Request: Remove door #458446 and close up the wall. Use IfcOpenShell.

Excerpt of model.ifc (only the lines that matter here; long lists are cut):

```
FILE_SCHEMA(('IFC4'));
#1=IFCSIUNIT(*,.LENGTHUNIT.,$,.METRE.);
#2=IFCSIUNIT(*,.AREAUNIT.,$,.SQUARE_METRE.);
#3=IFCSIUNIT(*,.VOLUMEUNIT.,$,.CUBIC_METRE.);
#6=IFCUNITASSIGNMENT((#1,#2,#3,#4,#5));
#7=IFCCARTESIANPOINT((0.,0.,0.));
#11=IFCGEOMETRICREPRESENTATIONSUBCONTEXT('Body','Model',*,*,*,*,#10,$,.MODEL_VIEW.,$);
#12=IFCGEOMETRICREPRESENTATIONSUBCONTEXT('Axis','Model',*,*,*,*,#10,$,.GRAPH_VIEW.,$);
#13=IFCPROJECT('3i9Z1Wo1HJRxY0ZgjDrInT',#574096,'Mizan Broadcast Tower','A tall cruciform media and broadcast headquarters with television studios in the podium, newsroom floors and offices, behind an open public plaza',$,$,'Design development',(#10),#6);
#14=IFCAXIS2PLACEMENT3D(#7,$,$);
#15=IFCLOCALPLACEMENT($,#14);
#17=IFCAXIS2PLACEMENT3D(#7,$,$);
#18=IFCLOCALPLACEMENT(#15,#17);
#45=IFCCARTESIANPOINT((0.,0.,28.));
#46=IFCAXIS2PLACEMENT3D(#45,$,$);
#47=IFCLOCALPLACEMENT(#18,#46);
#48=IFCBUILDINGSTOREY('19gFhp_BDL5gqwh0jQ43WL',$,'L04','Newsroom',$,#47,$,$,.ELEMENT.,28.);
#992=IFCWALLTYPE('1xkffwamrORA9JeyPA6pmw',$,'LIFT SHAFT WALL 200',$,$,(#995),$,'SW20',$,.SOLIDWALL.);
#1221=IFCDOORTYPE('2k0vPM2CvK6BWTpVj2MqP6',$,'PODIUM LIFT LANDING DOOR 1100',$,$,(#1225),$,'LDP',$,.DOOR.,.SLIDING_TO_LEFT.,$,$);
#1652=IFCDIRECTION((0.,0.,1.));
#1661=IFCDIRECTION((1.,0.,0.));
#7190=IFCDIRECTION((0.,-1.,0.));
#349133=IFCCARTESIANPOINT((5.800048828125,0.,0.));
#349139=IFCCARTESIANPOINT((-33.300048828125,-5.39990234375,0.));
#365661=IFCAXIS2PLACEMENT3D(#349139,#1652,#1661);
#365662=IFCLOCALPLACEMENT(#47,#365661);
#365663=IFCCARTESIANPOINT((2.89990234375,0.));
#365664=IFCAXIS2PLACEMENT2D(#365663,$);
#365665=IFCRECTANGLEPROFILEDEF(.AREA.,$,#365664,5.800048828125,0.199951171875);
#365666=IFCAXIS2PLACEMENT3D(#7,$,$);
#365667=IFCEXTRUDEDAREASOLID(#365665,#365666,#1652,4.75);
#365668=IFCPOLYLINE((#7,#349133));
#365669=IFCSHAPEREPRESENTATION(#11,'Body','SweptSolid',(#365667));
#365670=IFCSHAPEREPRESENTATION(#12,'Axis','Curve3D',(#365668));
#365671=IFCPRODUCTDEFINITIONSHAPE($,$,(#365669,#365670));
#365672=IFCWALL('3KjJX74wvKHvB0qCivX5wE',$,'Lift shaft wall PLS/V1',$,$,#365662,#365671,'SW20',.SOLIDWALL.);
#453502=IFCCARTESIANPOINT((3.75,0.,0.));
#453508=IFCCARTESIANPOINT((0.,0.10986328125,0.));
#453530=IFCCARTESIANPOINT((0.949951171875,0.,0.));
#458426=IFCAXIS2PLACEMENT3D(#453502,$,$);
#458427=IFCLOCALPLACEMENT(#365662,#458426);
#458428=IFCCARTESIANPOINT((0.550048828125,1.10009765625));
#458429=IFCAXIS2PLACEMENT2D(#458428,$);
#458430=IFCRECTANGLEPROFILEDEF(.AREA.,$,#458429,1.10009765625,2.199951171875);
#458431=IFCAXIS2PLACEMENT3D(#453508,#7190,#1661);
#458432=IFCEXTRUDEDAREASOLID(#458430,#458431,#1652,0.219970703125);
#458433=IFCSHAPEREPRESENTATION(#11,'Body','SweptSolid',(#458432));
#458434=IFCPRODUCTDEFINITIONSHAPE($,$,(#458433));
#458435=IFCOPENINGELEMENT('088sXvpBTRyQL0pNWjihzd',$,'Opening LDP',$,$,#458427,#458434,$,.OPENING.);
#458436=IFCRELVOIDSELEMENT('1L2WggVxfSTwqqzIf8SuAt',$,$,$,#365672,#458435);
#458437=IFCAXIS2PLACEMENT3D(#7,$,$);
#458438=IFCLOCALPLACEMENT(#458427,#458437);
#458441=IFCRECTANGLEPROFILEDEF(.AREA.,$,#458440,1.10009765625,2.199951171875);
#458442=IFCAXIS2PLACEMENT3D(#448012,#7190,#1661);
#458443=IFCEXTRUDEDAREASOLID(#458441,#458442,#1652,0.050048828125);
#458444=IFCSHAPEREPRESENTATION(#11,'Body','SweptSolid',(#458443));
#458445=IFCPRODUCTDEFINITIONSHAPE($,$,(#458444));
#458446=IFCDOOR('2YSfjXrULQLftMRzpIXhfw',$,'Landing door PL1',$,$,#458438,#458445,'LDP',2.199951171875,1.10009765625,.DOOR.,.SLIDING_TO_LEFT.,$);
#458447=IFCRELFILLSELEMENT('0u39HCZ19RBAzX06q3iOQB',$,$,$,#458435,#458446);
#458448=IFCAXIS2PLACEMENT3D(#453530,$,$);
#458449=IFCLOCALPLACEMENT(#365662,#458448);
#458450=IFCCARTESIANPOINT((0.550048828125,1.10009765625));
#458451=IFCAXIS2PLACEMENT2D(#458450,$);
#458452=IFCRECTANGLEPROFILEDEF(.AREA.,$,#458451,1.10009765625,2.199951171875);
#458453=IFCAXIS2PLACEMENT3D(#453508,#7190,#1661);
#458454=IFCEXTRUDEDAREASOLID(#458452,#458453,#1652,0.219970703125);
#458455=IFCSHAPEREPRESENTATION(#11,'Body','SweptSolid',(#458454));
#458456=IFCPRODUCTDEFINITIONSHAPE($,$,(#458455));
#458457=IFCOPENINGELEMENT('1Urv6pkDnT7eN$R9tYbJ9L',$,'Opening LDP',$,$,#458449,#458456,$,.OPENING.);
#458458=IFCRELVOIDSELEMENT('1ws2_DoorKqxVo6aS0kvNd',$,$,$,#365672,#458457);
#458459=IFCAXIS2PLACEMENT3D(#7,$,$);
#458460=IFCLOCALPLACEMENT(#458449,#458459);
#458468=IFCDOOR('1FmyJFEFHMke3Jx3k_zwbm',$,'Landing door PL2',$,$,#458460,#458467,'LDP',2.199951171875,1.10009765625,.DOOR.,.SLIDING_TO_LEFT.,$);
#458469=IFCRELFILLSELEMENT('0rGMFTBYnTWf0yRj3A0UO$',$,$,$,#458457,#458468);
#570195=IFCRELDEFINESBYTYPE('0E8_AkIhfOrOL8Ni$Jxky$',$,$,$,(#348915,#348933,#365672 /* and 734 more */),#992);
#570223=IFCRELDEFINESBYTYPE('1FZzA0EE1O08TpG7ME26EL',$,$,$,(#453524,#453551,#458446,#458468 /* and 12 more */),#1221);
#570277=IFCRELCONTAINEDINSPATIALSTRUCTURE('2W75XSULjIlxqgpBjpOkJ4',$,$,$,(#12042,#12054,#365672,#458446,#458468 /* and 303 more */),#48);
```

```python
import ifcopenshell
import ifcopenshell.api.feature
import ifcopenshell.api.root
import ifcopenshell.geom
import ifcopenshell.util.shape

model = ifcopenshell.open("model.ifc")
settings = ifcopenshell.geom.settings()


def volume(element):
    """Net volume in cubic metres, openings subtracted."""
    shape = ifcopenshell.geom.create_shape(settings, element)
    return ifcopenshell.util.shape.get_volume(shape.geometry)


door = model.by_guid("2YSfjXrULQLftMRzpIXhfw")
opening = door.FillsVoids[0].RelatingOpeningElement
wall = opening.VoidsElements[0].RelatingBuildingElement
before = volume(wall)

ifcopenshell.api.root.remove_product(model, product=door)
ifcopenshell.api.feature.remove_feature(model, feature=opening)

after = volume(wall)

print(f"wall volume {before:.3f} -> {after:.3f} m3")

model.write("model_rev.ifc")
```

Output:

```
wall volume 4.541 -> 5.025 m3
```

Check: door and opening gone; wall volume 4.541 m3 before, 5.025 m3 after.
